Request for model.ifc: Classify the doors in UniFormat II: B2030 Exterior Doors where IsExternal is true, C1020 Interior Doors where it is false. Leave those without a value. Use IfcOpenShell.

First a look at what the model holds.

```python
import ifcopenshell
import ifcopenshell.util.element

model = ifcopenshell.open("model.ifc")
print(model.schema)
print("classifications:", [c.Name for c in model.by_type("IfcClassification")])
values = [ifcopenshell.util.element.get_pset(e, "Pset_DoorCommon", "IsExternal") for e in model.by_type("IfcDoor")]
for value in (True, False, None):
    print("IsExternal", value, values.count(value))
```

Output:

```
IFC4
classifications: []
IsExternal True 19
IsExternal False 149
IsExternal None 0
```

```python
import ifcopenshell
import ifcopenshell.api.classification
import ifcopenshell.util.element

model = ifcopenshell.open("model.ifc")

system = ifcopenshell.api.classification.add_classification(model, classification="UniFormat II")

doors = model.by_type("IfcDoor")
external = {e: ifcopenshell.util.element.get_pset(e, "Pset_DoorCommon", "IsExternal") for e in doors}
for flag, code, name in ((True, "B2030", "Exterior Doors"), (False, "C1020", "Interior Doors")):
    products = [e for e in doors if external[e] is flag]
    ifcopenshell.api.classification.add_reference(
        model, products=products, classification=system, identification=code, name=name
    )
    print(code, len(products))

model.write("model_updated.ifc")
```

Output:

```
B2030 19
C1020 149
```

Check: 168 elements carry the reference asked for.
